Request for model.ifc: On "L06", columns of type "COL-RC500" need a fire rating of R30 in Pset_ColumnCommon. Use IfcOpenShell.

First a look at what the model holds.

```python
import ifcopenshell
import ifcopenshell.util.element

model = ifcopenshell.open("model.ifc")
print(model.schema)
storey = next(s for s in model.by_type("IfcBuildingStorey") if s.Name == "L06")
columns = [e for e in ifcopenshell.util.element.get_decomposition(storey) if e.is_a("IfcColumn")]
seen = {}
for e in columns:
    element_type = ifcopenshell.util.element.get_type(e)
    key = (element_type.Name if element_type != e and element_type else None, ifcopenshell.util.element.get_pset(e, "Pset_ColumnCommon", "FireRating"))
    seen[key] = seen.get(key, 0) + 1
for (name, value), count in sorted(seen.items(), key=str):
    print(count, "x", name, "|", value)
```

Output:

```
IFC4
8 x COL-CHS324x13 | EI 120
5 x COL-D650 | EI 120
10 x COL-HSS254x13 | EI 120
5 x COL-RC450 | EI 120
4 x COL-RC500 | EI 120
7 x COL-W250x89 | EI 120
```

```python
import ifcopenshell
import ifcopenshell.api.pset
import ifcopenshell.util.element

model = ifcopenshell.open("model.ifc")

storey = next(s for s in model.by_type("IfcBuildingStorey") if s.Name == "L06")
columns = [e for e in ifcopenshell.util.element.get_decomposition(storey) if e.is_a("IfcColumn")]

count = 0
for e in columns:
    element_type = ifcopenshell.util.element.get_type(e)
    if element_type in (None, e) or element_type.Name != "COL-RC500":
        continue
    # add_pset returns the element's existing set when there is one.
    pset = ifcopenshell.api.pset.add_pset(model, product=e, name="Pset_ColumnCommon")
    ifcopenshell.api.pset.edit_pset(model, pset=pset, properties={"FireRating": "R30"})
    count += 1

print(count, "columns updated")

model.write("model_rev.ifc")
```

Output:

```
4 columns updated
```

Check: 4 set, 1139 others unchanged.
